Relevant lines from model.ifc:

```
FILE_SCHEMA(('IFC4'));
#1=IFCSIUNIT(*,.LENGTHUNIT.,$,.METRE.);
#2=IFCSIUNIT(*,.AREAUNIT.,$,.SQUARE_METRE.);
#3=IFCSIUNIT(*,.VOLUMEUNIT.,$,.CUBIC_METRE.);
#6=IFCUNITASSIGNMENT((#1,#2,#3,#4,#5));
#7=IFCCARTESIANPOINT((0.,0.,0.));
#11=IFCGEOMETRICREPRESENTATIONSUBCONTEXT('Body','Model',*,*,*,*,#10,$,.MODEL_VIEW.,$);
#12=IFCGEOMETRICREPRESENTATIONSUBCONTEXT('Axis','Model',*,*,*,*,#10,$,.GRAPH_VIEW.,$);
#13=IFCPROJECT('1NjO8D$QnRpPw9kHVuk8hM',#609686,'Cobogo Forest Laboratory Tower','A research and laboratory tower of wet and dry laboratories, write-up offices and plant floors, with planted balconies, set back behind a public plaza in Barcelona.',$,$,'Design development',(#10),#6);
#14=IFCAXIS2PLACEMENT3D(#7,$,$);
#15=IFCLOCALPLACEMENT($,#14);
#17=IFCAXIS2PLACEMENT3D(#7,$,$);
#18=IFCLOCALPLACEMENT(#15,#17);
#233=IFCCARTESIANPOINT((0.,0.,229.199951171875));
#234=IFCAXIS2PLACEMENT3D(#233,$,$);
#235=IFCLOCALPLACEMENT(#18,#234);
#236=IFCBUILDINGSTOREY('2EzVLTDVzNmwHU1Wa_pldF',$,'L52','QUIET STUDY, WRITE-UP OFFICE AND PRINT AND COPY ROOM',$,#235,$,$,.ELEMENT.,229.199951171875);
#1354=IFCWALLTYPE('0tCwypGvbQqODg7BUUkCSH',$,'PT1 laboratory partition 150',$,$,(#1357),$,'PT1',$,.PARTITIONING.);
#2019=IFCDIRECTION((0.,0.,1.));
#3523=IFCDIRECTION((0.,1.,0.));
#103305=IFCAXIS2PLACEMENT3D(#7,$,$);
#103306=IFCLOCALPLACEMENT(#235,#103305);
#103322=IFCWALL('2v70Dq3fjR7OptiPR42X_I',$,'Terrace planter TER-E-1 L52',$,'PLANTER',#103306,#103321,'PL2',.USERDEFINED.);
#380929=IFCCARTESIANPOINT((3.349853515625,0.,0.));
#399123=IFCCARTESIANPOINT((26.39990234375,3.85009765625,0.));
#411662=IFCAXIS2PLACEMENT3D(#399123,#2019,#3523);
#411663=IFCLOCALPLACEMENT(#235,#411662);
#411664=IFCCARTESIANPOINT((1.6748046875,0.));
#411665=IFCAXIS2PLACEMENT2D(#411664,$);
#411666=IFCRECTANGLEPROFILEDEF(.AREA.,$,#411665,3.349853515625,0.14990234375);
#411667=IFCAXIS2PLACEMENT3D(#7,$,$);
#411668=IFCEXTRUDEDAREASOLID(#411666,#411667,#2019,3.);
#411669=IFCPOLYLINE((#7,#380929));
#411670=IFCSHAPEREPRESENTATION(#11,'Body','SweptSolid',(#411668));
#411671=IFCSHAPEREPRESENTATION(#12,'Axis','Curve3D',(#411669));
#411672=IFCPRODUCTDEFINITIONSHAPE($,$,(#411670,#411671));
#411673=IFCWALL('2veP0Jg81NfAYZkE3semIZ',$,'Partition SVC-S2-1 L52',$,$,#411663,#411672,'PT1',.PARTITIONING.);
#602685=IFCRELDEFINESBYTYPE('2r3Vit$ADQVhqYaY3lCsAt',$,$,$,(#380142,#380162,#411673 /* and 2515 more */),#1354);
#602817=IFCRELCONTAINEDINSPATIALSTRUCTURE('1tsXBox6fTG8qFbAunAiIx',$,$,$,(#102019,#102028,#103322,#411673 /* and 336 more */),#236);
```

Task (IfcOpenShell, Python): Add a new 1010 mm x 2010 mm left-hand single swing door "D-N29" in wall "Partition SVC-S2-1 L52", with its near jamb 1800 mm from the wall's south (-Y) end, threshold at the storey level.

```python
import numpy as np
import ifcopenshell
import ifcopenshell.api.feature
import ifcopenshell.api.geometry
import ifcopenshell.api.root
import ifcopenshell.api.spatial
import ifcopenshell.geom
import ifcopenshell.util.element
import ifcopenshell.util.placement
import ifcopenshell.util.representation
import ifcopenshell.util.shape
import ifcopenshell.util.unit

model = ifcopenshell.open("model.ifc")
unit_scale = ifcopenshell.util.unit.calculate_unit_scale(model)
settings = ifcopenshell.geom.settings()


def volume(element):
    """Net volume in cubic metres, openings subtracted."""
    shape = ifcopenshell.geom.create_shape(settings, element)
    return ifcopenshell.util.shape.get_volume(shape.geometry)


wall = model.by_guid("2veP0Jg81NfAYZkE3semIZ")
storey = ifcopenshell.util.element.get_container(wall, ifc_class="IfcBuildingStorey")
context = ifcopenshell.util.representation.get_context(model, "Model", "Body", "MODEL_VIEW")
before = volume(wall)

width, height, from_end, sill = 1.01, 2.01, 1.8, 0.0  # metres

# The wall runs along its own X axis, and the end named is its -X end.
wall_shape = ifcopenshell.geom.create_shape(settings, wall)
x, y, z = ifcopenshell.util.shape.get_vertices(wall_shape.geometry).T
start = x.min() + from_end
face, thickness = float(y.min()), float(y.max() - y.min())
wall_matrix = ifcopenshell.util.placement.get_local_placement(wall.ObjectPlacement)
level = ifcopenshell.util.placement.get_local_placement(storey.ObjectPlacement)[2, 3]


def in_wall(x, y):
    """Placement at x, y metres in the wall's axes, at sill height."""
    matrix = wall_matrix.copy()
    matrix[:, 3] = wall_matrix @ np.array([x / unit_scale, y / unit_scale, 0.0, 1.0])
    matrix[2, 3] = level + sill / unit_scale
    return matrix


# Opening: a box that overshoots both wall faces by 50 mm.
opening = ifcopenshell.api.root.create_entity(model, ifc_class="IfcOpeningElement", predefined_type="OPENING")
box = ifcopenshell.api.geometry.add_wall_representation(
    model, context=context, length=width, height=height, thickness=thickness + 0.1
)
ifcopenshell.api.geometry.assign_representation(model, product=opening, representation=box)
ifcopenshell.api.geometry.edit_object_placement(model, product=opening, matrix=in_wall(start, face - 0.05), is_si=False)
ifcopenshell.api.feature.add_feature(model, feature=opening, element=wall)

door = ifcopenshell.api.root.create_entity(model, ifc_class="IfcDoor", name="D-N29", predefined_type="DOOR")
door.OverallWidth, door.OverallHeight = width / unit_scale, height / unit_scale
door.OperationType = "SINGLE_SWING_LEFT"
body = ifcopenshell.api.geometry.add_door_representation(
    model,
    context=context,
    overall_width=door.OverallWidth,
    overall_height=door.OverallHeight,
    operation_type="SINGLE_SWING_LEFT",
    lining_properties={"LiningDepth": thickness / unit_scale, "ThresholdDepth": thickness / unit_scale},
)
ifcopenshell.api.geometry.assign_representation(model, product=door, representation=body)
ifcopenshell.api.spatial.assign_container(model, products=[door], relating_structure=storey)
ifcopenshell.api.feature.add_filling(model, opening=opening, element=door)

# The lining spans the wall, so the door starts at the wall face.
ifcopenshell.api.geometry.edit_object_placement(model, product=door, matrix=in_wall(start, face), is_si=False)

after = volume(wall)

print(f"wall volume {before:.3f} -> {after:.3f} m3")

model.write("model_v2.ifc")
```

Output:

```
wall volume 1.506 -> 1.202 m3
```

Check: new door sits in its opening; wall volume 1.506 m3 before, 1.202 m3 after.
